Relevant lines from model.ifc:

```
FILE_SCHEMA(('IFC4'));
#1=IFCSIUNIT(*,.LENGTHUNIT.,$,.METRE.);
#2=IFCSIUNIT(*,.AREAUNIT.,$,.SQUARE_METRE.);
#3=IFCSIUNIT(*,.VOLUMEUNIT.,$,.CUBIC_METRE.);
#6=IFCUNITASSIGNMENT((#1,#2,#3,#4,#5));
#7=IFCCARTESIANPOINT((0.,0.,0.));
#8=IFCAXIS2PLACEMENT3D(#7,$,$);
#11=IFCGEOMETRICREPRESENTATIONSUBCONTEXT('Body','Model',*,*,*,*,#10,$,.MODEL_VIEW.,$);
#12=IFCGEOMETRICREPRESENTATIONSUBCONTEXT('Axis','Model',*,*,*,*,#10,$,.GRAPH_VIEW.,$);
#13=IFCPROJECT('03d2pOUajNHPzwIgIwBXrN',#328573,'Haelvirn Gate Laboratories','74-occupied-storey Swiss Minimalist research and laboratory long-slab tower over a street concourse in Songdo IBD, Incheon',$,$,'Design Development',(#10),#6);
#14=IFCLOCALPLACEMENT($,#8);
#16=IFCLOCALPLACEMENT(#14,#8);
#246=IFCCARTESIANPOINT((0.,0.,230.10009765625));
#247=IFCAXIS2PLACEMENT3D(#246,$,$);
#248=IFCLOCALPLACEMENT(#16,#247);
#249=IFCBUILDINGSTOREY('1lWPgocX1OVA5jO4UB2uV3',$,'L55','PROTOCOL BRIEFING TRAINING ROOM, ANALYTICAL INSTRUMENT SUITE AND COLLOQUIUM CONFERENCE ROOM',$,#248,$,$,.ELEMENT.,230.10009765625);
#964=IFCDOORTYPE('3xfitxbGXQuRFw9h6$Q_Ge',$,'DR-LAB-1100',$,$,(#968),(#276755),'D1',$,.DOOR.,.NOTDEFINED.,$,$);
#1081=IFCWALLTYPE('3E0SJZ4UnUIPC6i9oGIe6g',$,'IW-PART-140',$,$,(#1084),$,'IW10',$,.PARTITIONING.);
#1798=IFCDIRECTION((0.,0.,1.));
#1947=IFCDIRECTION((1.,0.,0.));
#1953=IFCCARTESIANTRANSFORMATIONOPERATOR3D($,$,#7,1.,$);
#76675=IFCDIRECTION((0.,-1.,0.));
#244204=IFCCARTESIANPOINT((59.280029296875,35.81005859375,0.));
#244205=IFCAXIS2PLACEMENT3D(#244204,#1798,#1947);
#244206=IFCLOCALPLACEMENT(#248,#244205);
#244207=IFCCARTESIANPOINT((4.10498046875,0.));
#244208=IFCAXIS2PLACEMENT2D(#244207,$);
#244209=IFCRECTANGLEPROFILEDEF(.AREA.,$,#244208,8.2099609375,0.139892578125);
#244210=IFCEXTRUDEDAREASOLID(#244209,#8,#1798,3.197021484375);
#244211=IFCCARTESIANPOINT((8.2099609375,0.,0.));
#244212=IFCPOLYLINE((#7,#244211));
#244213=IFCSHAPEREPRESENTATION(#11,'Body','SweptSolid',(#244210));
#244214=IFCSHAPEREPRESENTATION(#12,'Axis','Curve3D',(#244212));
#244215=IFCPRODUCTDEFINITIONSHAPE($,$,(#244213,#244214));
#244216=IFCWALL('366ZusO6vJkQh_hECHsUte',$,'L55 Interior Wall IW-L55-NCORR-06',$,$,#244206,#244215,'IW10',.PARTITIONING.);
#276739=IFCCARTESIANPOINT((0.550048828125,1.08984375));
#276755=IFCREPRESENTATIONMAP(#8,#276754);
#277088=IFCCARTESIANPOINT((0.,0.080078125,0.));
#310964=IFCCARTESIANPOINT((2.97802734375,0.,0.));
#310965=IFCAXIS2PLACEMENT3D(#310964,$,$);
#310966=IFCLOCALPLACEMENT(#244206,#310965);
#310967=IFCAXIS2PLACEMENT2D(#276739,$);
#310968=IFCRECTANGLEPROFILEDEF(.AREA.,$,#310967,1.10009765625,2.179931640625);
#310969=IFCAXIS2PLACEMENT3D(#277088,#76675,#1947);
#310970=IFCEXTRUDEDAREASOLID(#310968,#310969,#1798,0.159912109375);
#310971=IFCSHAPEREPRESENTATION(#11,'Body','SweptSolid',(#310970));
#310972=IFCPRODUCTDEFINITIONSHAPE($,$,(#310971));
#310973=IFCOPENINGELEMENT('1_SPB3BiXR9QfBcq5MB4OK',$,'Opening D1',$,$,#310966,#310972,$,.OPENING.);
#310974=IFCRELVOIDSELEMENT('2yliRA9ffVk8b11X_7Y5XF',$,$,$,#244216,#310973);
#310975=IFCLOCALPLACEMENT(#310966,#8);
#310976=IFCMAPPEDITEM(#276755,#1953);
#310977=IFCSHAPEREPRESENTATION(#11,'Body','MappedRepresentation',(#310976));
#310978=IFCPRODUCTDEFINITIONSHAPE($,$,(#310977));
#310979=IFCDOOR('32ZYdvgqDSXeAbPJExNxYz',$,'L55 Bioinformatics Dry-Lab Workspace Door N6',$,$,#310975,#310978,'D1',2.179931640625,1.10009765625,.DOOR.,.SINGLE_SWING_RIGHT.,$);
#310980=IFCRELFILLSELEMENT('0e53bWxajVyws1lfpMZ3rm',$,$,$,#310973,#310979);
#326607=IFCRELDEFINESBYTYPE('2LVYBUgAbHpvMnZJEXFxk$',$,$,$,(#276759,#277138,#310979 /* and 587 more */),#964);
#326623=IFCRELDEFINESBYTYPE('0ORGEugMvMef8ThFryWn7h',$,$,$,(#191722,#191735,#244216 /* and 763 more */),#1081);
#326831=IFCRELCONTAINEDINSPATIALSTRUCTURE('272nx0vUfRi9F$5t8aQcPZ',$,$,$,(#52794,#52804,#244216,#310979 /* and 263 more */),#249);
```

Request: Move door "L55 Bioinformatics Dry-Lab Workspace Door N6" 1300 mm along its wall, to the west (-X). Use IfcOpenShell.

```python
import ifcopenshell
import ifcopenshell.api.geometry
import ifcopenshell.util.placement
import ifcopenshell.util.unit

model = ifcopenshell.open("model.ifc")
unit_scale = ifcopenshell.util.unit.calculate_unit_scale(model)

door = model.by_guid("32ZYdvgqDSXeAbPJExNxYz")
opening = door.FillsVoids[0].RelatingOpeningElement
wall = opening.VoidsElements[0].RelatingBuildingElement

wall_matrix = ifcopenshell.util.placement.get_local_placement(wall.ObjectPlacement)
shift = wall_matrix[:3, 0] * -1.3 / unit_scale
before = ifcopenshell.util.placement.get_local_placement(door.ObjectPlacement)[:3, 3].copy()

# The door is placed relative to its opening, so it follows when the opening moves.
matrix = ifcopenshell.util.placement.get_local_placement(opening.ObjectPlacement)
matrix[:3, 3] += shift
ifcopenshell.api.geometry.edit_object_placement(
    model, product=opening, matrix=matrix, is_si=False, should_transform_children=True
)

after = ifcopenshell.util.placement.get_local_placement(door.ObjectPlacement)[:3, 3]
print("door moved by", (after - before).round(3) + 0.0)

model.write("model-out.ifc")
```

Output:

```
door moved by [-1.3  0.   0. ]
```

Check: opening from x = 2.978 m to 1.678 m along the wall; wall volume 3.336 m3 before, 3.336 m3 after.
